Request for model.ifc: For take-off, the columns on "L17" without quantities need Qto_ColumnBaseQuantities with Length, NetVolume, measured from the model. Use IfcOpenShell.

First a look at what the model holds.

```python
import ifcopenshell
import ifcopenshell.util.element
import ifcopenshell.util.unit

model = ifcopenshell.open("model.ifc")
print(model.schema)
for unit_type in ("LENGTHUNIT", "AREAUNIT", "VOLUMEUNIT"):
    print(unit_type, ifcopenshell.util.unit.calculate_unit_scale(model, unit_type))
storey = next(s for s in model.by_type("IfcBuildingStorey") if s.Name == "L17")
columns = [e for e in ifcopenshell.util.element.get_decomposition(storey) if e.is_a("IfcColumn")]
for e in sorted(columns, key=lambda e: e.id()):
    print(e.id(), e.is_a(), e.Name, list(ifcopenshell.util.element.get_psets(e, qtos_only=True)), sep=" | ")
```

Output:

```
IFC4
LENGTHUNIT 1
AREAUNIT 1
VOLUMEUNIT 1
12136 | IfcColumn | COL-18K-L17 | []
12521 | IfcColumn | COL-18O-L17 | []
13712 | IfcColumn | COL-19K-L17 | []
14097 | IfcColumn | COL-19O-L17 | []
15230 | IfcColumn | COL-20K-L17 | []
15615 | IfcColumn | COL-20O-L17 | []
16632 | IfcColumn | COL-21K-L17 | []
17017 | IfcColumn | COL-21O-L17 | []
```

```python
import ifcopenshell
import ifcopenshell.api.pset
import ifcopenshell.geom
import ifcopenshell.util.element
import ifcopenshell.util.shape
import ifcopenshell.util.unit

model = ifcopenshell.open("model.ifc")
unit_scale = ifcopenshell.util.unit.calculate_unit_scale(model)
volume_scale = ifcopenshell.util.unit.calculate_unit_scale(model, "VOLUMEUNIT")
settings = ifcopenshell.geom.settings()

storey = next(s for s in model.by_type("IfcBuildingStorey") if s.Name == "L17")
columns = [e for e in ifcopenshell.util.element.get_decomposition(storey) if e.is_a("IfcColumn")]

for e in sorted(columns, key=lambda e: e.id()):
    if ifcopenshell.util.element.get_psets(e, qtos_only=True, should_inherit=False):
        continue
    # Geometry comes back in metres, in the element's own axes.
    shape = ifcopenshell.geom.create_shape(settings, e)
    values = {
        "Length": ifcopenshell.util.shape.get_z(shape.geometry) / unit_scale,
        "NetVolume": ifcopenshell.util.shape.get_volume(shape.geometry) / volume_scale,
    }
    qto = ifcopenshell.api.pset.add_qto(model, product=e, name="Qto_ColumnBaseQuantities")
    ifcopenshell.api.pset.edit_qto(model, qto=qto, properties=values)
    print(e.id(), {k: round(v, 3) for k, v in values.items()})

model.write("model_updated.ifc")
```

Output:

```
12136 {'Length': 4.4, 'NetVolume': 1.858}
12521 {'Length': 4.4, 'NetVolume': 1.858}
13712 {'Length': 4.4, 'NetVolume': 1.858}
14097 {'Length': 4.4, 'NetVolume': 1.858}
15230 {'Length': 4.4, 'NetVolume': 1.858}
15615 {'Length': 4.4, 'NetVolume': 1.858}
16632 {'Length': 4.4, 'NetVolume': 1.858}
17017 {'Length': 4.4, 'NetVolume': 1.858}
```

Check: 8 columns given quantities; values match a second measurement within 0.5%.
